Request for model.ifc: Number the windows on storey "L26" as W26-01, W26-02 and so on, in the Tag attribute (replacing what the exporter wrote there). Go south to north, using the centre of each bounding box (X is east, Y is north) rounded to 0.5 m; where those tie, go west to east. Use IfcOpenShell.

First a look at what the model holds.

```python
import ifcopenshell
import ifcopenshell.util.element
import ifcopenshell.util.placement

model = ifcopenshell.open("model.ifc")
print(model.schema)
storey = next(s for s in model.by_type("IfcBuildingStorey") if s.Name == "L26")
windows = [e for e in ifcopenshell.util.element.get_decomposition(storey) if e.is_a("IfcWindow")]
for e in sorted(windows, key=lambda e: e.id()):
    origin = ifcopenshell.util.placement.get_local_placement(e.ObjectPlacement)[:3, 3]
    print(e.id(), e.Tag, e.Name, origin.round(2) + 0.0, sep=" | ")
```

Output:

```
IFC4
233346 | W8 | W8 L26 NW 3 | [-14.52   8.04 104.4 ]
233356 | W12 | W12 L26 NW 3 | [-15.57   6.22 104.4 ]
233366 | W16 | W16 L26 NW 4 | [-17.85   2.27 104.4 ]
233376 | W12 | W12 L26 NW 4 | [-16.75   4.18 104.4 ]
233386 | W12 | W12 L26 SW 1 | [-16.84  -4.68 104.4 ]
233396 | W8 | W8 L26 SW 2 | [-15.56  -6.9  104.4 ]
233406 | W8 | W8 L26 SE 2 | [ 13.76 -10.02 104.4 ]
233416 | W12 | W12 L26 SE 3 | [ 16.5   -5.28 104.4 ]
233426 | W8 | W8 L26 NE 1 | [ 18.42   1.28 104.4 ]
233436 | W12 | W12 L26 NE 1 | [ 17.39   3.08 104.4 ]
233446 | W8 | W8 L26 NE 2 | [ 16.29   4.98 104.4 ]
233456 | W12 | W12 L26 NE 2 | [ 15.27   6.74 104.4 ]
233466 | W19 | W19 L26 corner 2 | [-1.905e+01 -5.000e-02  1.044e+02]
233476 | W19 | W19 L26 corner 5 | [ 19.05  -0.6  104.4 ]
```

```python
import ifcopenshell
import ifcopenshell.geom
import ifcopenshell.util.element
import ifcopenshell.util.shape

model = ifcopenshell.open("model.ifc")
settings = ifcopenshell.geom.settings()
settings.set("use-world-coords", True)


def centre(element):
    shape = ifcopenshell.geom.create_shape(settings, element)
    return ifcopenshell.util.shape.get_bbox_centroid(shape.geometry)


storey = next(s for s in model.by_type("IfcBuildingStorey") if s.Name == "L26")
windows = [e for e in ifcopenshell.util.element.get_decomposition(storey) if e.is_a("IfcWindow")]

# Insertion points can sit at a corner or the storey origin, so sort by the geometry (in metres).
centres = {e: centre(e) for e in windows}
windows.sort(key=lambda e: (round(centres[e][1] / 0.5), centres[e][0]))

for i, e in enumerate(windows, start=1):
    number = f"W26-{i:02d}"
    e.Tag = number
    print(e.id(), number)

model.write("model_edited.ifc")
```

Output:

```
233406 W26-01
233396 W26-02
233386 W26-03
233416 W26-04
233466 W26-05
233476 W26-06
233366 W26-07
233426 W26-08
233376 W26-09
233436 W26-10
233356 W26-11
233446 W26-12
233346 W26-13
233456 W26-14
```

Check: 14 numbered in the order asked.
